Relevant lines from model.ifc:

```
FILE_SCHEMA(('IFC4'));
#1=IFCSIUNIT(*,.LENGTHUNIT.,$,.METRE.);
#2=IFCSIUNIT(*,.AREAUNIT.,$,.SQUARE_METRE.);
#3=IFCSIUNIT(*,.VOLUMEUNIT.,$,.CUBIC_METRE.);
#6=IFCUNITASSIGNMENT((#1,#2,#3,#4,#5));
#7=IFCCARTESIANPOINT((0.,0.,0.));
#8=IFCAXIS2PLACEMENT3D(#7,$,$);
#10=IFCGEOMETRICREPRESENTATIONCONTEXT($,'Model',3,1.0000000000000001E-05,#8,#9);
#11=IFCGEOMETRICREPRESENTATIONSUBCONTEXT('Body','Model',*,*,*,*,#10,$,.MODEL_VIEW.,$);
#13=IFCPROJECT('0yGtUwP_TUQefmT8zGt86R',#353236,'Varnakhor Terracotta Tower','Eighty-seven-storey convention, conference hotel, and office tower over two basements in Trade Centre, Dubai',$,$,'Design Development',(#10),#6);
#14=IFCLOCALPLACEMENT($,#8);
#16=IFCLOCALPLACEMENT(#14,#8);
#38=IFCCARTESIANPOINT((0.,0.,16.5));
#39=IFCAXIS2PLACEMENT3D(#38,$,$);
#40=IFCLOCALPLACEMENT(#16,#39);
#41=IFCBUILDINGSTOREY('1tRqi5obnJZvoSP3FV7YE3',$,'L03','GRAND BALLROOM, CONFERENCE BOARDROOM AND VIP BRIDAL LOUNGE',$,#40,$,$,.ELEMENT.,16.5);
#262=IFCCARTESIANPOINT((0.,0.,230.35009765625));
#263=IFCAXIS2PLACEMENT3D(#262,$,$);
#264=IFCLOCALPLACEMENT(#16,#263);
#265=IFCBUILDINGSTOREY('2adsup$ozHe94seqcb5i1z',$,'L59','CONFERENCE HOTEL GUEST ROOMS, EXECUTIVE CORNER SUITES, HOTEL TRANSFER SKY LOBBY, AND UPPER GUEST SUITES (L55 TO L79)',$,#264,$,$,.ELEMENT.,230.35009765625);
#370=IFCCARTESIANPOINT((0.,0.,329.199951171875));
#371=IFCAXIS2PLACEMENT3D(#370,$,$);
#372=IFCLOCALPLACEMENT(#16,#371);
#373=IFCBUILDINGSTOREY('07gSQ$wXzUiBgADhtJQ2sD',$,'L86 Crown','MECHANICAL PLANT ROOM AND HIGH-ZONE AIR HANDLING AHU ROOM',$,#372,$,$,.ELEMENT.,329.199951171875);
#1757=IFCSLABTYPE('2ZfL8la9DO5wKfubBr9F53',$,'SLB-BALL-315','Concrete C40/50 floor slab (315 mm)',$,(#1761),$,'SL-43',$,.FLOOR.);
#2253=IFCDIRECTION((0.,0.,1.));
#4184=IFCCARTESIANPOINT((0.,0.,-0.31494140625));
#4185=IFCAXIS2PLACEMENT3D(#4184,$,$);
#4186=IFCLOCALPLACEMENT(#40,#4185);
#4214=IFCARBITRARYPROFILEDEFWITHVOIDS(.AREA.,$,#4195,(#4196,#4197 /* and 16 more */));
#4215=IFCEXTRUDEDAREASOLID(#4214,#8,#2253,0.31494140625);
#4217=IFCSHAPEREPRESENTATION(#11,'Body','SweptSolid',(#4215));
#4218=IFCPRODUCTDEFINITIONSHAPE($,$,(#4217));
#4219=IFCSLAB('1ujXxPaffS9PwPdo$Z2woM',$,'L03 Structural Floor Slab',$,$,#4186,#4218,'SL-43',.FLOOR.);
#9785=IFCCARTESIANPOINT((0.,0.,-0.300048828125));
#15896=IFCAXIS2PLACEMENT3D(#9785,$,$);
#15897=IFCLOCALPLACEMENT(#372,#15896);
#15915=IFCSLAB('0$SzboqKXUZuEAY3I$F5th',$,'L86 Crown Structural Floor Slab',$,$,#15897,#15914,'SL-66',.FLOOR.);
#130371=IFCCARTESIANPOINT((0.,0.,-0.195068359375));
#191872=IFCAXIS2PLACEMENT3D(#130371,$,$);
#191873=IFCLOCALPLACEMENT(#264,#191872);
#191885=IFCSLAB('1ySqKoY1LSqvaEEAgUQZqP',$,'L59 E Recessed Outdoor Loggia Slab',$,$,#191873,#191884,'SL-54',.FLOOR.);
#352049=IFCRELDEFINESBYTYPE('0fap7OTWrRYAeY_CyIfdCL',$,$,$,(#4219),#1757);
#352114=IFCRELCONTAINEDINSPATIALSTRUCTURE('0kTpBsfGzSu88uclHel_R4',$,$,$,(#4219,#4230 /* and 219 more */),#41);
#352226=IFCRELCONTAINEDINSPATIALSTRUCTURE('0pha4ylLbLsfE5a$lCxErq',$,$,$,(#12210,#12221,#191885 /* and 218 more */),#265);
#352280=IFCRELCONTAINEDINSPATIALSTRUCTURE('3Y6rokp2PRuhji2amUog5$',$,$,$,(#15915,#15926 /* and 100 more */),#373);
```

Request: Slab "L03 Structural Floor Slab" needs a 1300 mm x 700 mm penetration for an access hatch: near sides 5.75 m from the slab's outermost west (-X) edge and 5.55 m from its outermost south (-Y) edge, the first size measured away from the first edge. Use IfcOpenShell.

```python
import numpy as np
import ifcopenshell
import ifcopenshell.api.feature
import ifcopenshell.api.geometry
import ifcopenshell.api.root
import ifcopenshell.geom
import ifcopenshell.util.placement
import ifcopenshell.util.representation
import ifcopenshell.util.shape
import ifcopenshell.util.unit

model = ifcopenshell.open("model.ifc")
unit_scale = ifcopenshell.util.unit.calculate_unit_scale(model)
settings = ifcopenshell.geom.settings()


def volume(element):
    """Net volume in cubic metres, openings subtracted."""
    shape = ifcopenshell.geom.create_shape(settings, element)
    return ifcopenshell.util.shape.get_volume(shape.geometry)


slab = model.by_guid("1ujXxPaffS9PwPdo$Z2woM")
before = volume(slab)

# Extent in the slab's own axes, in metres. The edges named are its -X and -Y sides.
slab_shape = ifcopenshell.geom.create_shape(settings, slab)
vertices = ifcopenshell.util.shape.get_vertices(slab_shape.geometry)
x_min, y_min, bottom = vertices.min(axis=0)
top = vertices[:, 2].max()

opening = ifcopenshell.api.root.create_entity(model, ifc_class="IfcOpeningElement", name="Access hatch opening", predefined_type="OPENING")
context = ifcopenshell.util.representation.get_context(model, "Model", "Body", "MODEL_VIEW")
width, depth = 1.3, 0.7
outline = [(0.0, 0.0), (width, 0.0), (width, depth), (0.0, depth), (0.0, 0.0)]
# Overshoot both faces by 50 mm so the cut is clean.
shape = ifcopenshell.api.geometry.add_slab_representation(
    model, context=context, depth=top - bottom + 0.1, polyline=outline
)
ifcopenshell.api.geometry.assign_representation(model, product=opening, representation=shape)

matrix = ifcopenshell.util.placement.get_local_placement(slab.ObjectPlacement)
matrix[:, 3] = matrix @ np.append(np.array([x_min + 5.75, y_min + 5.55, bottom - 0.05]) / unit_scale, 1.0)
ifcopenshell.api.geometry.edit_object_placement(model, product=opening, matrix=matrix, is_si=False)
ifcopenshell.api.feature.add_feature(model, feature=opening, element=slab)

after = volume(slab)

print(f"slab volume {before:.3f} -> {after:.3f} m3")

model.write("model_updated.ifc")
```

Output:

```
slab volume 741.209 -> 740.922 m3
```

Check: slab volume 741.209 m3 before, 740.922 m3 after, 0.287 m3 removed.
